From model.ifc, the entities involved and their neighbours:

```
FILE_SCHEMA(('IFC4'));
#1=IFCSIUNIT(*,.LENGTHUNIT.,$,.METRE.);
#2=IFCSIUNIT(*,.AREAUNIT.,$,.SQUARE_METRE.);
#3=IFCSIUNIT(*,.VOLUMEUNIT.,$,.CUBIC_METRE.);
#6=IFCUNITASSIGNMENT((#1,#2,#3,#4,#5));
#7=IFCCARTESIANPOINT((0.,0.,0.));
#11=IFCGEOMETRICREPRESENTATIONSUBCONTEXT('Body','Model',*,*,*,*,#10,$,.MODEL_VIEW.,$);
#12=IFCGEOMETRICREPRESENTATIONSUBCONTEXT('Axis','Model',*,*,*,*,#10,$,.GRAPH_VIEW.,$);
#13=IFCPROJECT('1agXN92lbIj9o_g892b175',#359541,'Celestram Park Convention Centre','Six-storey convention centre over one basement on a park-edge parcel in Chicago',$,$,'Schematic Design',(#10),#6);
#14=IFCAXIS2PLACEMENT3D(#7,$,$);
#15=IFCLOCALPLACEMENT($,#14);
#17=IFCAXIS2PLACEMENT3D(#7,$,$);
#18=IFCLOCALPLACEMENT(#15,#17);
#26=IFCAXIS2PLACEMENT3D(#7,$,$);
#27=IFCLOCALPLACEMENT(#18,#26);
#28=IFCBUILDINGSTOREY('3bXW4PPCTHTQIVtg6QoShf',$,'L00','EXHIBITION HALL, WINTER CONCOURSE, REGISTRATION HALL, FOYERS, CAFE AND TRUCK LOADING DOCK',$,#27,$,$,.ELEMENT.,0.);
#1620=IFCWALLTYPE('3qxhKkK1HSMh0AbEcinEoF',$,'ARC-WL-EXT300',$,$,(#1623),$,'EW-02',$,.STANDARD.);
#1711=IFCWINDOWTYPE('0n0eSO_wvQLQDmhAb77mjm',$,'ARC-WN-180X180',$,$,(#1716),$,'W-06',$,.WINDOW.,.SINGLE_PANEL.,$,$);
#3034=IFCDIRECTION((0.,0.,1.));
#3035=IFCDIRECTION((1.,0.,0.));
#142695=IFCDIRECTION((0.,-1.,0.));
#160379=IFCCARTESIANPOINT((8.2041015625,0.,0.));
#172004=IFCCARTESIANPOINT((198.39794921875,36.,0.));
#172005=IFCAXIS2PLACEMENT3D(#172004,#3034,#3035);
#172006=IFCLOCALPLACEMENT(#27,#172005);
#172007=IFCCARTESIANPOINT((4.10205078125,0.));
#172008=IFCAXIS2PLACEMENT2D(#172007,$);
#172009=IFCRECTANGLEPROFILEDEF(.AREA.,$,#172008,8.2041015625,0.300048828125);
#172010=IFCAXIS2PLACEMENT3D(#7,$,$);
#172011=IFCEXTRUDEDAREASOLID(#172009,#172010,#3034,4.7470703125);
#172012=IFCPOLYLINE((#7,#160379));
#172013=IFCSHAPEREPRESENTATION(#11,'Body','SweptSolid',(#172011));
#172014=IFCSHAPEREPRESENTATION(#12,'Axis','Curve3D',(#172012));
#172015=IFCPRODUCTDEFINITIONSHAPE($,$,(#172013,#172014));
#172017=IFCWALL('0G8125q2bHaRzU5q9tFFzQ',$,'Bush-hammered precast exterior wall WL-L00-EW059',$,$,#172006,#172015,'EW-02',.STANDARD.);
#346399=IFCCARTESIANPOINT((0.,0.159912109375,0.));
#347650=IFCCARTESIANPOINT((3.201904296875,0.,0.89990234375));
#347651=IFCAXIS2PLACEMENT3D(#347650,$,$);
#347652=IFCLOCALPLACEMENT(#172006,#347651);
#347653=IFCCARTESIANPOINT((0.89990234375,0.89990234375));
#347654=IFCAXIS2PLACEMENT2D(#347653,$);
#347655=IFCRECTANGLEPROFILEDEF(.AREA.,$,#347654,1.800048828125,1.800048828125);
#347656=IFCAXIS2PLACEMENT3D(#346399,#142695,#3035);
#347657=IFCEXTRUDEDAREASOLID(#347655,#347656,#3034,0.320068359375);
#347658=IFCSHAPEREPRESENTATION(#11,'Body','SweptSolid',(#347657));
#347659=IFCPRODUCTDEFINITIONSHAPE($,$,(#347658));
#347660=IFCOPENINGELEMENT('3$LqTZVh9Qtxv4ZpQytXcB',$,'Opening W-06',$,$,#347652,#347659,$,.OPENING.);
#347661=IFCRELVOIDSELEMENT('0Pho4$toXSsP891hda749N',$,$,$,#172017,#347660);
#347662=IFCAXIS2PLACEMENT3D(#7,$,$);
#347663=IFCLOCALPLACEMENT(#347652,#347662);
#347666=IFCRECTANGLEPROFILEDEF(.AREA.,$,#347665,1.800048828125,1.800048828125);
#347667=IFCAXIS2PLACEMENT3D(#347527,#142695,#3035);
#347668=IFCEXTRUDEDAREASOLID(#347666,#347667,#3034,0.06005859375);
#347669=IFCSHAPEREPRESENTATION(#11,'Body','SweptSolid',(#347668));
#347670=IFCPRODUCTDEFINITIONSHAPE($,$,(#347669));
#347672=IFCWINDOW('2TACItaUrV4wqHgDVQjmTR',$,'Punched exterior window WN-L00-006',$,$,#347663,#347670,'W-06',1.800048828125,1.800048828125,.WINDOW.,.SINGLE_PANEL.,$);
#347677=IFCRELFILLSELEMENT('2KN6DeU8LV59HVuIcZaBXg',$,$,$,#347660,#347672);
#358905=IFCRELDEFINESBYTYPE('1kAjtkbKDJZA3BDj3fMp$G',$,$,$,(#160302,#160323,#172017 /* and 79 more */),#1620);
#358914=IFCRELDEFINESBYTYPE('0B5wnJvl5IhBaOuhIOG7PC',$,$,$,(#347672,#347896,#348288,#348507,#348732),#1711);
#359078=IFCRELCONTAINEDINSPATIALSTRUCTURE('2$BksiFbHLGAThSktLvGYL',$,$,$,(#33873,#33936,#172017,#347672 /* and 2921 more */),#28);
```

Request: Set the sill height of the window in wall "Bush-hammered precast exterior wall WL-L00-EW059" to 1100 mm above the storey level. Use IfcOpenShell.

```python
import numpy as np
import ifcopenshell
import ifcopenshell.api.geometry
import ifcopenshell.geom
import ifcopenshell.util.element
import ifcopenshell.util.placement
import ifcopenshell.util.shape
import ifcopenshell.util.unit

model = ifcopenshell.open("model.ifc")
unit_scale = ifcopenshell.util.unit.calculate_unit_scale(model)

window = model.by_id(347672)
opening = window.FillsVoids[0].RelatingOpeningElement
storey = ifcopenshell.util.element.get_container(window, ifc_class="IfcBuildingStorey")
level = ifcopenshell.util.placement.get_local_placement(storey.ObjectPlacement)[2, 3]

# The opening's origin need not be at the sill, so measure its lowest point.
shape = ifcopenshell.geom.create_shape(ifcopenshell.geom.settings(), opening)
bottom = ifcopenshell.util.shape.get_shape_bottom_elevation(shape, shape.geometry) / unit_scale
dz = level + 1.1 / unit_scale - bottom

shift = np.array([0.0, 0.0, dz])
# The window is placed relative to its opening, so it follows when the opening moves.
matrix = ifcopenshell.util.placement.get_local_placement(opening.ObjectPlacement)
matrix[:3, 3] += shift
ifcopenshell.api.geometry.edit_object_placement(
    model, product=opening, matrix=matrix, is_si=False, should_transform_children=True
)

print(f"moved by {dz * unit_scale:+.3f} m")

model.write("model-out.ifc")
```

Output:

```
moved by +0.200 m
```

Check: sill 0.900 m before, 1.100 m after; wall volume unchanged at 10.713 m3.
